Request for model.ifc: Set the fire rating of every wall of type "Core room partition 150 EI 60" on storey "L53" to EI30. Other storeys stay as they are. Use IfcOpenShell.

First a look at what the model holds.

```python
import ifcopenshell
import ifcopenshell.util.element

model = ifcopenshell.open("model.ifc")
print(model.schema)
storey = next(s for s in model.by_type("IfcBuildingStorey") if s.Name == "L53")
walls = [e for e in ifcopenshell.util.element.get_decomposition(storey) if e.is_a("IfcWall")]
seen = {}
for e in walls:
    element_type = ifcopenshell.util.element.get_type(e)
    key = (element_type.Name if element_type != e and element_type else None, ifcopenshell.util.element.get_pset(e, "Pset_WallCommon", "FireRating"))
    seen[key] = seen.get(key, 0) + 1
for (name, value), count in sorted(seen.items(), key=str):
    print(count, "x", name, "|", value)
```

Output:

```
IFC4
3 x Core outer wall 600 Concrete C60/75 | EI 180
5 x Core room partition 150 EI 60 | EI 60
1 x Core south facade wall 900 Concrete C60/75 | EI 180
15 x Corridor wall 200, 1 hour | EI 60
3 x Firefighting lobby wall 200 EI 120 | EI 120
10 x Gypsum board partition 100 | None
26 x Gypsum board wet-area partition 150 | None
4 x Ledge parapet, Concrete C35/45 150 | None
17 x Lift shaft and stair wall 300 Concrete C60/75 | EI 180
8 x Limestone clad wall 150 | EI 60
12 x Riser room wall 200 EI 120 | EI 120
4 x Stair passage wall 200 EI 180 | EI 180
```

```python
import ifcopenshell
import ifcopenshell.api.pset
import ifcopenshell.util.element

model = ifcopenshell.open("model.ifc")

storey = next(s for s in model.by_type("IfcBuildingStorey") if s.Name == "L53")
walls = [e for e in ifcopenshell.util.element.get_decomposition(storey) if e.is_a("IfcWall")]

count = 0
for e in walls:
    element_type = ifcopenshell.util.element.get_type(e)
    if element_type in (None, e) or element_type.Name != "Core room partition 150 EI 60":
        continue
    found = ifcopenshell.util.element.get_pset(e, "Pset_WallCommon", should_inherit=False)
    if found:
        pset = model.by_id(found["id"])
        if len(ifcopenshell.util.element.get_elements_by_pset(pset)) > 1:
            pset = ifcopenshell.api.pset.unshare_pset(model, products=[e], pset=pset)[0]
    else:
        pset = ifcopenshell.api.pset.add_pset(model, product=e, name="Pset_WallCommon")
    ifcopenshell.api.pset.edit_pset(model, pset=pset, properties={"FireRating": "EI30"})
    count += 1

print(count, "walls updated")

model.write("model-out.ifc")
```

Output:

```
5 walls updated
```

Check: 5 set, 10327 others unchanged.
